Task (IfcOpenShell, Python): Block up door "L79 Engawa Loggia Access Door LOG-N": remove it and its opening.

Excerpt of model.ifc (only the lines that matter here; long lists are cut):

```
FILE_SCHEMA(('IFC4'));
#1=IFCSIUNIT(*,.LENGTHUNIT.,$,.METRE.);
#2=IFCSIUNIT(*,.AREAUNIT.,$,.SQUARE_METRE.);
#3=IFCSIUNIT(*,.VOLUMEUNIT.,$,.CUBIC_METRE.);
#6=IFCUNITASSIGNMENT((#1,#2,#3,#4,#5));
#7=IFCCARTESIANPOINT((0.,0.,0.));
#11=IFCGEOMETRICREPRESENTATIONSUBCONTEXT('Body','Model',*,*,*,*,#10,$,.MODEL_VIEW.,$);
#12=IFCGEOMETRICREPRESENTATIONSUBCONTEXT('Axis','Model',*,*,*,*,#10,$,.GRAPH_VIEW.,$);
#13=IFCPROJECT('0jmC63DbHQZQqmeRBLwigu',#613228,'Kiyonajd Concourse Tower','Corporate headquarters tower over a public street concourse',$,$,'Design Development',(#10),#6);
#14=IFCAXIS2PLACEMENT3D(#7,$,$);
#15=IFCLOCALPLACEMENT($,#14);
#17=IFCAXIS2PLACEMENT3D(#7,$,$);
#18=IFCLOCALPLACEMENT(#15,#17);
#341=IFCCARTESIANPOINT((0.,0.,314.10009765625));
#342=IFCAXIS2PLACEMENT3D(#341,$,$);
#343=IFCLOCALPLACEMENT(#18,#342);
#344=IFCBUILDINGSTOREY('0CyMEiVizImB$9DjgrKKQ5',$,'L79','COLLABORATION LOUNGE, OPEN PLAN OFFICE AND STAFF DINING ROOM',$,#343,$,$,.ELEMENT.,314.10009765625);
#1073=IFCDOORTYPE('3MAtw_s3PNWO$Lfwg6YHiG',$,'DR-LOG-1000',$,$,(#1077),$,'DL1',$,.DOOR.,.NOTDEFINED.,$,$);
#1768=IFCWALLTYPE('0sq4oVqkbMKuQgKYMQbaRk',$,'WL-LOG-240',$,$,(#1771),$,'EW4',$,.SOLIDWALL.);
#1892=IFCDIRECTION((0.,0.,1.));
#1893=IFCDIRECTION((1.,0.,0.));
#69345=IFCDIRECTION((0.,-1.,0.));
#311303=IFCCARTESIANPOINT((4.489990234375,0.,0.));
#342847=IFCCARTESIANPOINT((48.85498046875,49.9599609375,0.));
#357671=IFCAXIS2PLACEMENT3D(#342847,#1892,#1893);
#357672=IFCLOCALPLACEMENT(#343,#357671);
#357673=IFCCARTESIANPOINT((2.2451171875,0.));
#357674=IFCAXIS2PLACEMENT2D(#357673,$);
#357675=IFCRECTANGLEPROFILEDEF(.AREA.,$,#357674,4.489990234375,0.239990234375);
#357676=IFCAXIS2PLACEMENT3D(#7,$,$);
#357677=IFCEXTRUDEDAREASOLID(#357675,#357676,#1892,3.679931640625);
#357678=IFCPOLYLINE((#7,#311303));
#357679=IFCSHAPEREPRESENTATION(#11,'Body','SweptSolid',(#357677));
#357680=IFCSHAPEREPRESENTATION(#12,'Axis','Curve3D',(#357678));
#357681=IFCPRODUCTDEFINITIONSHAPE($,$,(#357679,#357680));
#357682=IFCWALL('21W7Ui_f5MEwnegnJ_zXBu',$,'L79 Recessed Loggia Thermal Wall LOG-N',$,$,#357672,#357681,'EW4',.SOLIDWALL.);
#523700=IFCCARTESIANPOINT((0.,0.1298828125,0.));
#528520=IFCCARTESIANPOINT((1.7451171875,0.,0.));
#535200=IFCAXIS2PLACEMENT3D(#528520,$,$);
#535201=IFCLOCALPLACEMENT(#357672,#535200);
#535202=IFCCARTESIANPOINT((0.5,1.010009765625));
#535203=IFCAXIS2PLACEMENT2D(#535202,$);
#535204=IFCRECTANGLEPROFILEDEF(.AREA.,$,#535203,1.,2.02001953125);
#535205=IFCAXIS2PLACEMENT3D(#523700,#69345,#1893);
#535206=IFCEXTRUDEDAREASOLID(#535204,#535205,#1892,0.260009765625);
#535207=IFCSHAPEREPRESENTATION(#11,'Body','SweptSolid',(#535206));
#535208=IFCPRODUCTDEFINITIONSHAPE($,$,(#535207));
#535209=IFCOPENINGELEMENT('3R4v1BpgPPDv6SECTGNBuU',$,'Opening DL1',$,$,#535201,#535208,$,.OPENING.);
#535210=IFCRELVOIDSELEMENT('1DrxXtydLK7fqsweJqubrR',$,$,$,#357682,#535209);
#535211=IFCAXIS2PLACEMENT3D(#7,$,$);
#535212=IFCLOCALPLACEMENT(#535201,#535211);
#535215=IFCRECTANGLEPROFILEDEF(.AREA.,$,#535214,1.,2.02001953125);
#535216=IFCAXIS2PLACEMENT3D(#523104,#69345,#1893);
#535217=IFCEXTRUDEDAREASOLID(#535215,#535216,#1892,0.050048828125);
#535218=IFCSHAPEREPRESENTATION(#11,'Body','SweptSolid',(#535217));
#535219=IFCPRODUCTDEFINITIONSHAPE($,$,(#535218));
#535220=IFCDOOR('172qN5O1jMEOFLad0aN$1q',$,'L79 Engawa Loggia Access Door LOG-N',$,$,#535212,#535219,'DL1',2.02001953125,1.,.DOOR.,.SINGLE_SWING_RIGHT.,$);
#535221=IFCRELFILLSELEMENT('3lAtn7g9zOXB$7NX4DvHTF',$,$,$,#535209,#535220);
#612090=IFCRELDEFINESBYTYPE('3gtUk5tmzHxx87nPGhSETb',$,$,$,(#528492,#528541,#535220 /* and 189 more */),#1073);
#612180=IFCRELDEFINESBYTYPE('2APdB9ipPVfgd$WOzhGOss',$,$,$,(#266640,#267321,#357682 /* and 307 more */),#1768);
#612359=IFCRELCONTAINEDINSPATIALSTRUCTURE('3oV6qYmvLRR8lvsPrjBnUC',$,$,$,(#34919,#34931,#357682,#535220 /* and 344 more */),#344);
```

```python
import ifcopenshell
import ifcopenshell.api.feature
import ifcopenshell.api.root
import ifcopenshell.geom
import ifcopenshell.util.shape

model = ifcopenshell.open("model.ifc")
settings = ifcopenshell.geom.settings()


def volume(element):
    """Net volume in cubic metres, openings subtracted."""
    shape = ifcopenshell.geom.create_shape(settings, element)
    return ifcopenshell.util.shape.get_volume(shape.geometry)


door = model.by_guid("172qN5O1jMEOFLad0aN$1q")
opening = door.FillsVoids[0].RelatingOpeningElement
wall = opening.VoidsElements[0].RelatingBuildingElement
before = volume(wall)

ifcopenshell.api.root.remove_product(model, product=door)
ifcopenshell.api.feature.remove_feature(model, feature=opening)

after = volume(wall)

print(f"wall volume {before:.3f} -> {after:.3f} m3")

model.write("model-out.ifc")
```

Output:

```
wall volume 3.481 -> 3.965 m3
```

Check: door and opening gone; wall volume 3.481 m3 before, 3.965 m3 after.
